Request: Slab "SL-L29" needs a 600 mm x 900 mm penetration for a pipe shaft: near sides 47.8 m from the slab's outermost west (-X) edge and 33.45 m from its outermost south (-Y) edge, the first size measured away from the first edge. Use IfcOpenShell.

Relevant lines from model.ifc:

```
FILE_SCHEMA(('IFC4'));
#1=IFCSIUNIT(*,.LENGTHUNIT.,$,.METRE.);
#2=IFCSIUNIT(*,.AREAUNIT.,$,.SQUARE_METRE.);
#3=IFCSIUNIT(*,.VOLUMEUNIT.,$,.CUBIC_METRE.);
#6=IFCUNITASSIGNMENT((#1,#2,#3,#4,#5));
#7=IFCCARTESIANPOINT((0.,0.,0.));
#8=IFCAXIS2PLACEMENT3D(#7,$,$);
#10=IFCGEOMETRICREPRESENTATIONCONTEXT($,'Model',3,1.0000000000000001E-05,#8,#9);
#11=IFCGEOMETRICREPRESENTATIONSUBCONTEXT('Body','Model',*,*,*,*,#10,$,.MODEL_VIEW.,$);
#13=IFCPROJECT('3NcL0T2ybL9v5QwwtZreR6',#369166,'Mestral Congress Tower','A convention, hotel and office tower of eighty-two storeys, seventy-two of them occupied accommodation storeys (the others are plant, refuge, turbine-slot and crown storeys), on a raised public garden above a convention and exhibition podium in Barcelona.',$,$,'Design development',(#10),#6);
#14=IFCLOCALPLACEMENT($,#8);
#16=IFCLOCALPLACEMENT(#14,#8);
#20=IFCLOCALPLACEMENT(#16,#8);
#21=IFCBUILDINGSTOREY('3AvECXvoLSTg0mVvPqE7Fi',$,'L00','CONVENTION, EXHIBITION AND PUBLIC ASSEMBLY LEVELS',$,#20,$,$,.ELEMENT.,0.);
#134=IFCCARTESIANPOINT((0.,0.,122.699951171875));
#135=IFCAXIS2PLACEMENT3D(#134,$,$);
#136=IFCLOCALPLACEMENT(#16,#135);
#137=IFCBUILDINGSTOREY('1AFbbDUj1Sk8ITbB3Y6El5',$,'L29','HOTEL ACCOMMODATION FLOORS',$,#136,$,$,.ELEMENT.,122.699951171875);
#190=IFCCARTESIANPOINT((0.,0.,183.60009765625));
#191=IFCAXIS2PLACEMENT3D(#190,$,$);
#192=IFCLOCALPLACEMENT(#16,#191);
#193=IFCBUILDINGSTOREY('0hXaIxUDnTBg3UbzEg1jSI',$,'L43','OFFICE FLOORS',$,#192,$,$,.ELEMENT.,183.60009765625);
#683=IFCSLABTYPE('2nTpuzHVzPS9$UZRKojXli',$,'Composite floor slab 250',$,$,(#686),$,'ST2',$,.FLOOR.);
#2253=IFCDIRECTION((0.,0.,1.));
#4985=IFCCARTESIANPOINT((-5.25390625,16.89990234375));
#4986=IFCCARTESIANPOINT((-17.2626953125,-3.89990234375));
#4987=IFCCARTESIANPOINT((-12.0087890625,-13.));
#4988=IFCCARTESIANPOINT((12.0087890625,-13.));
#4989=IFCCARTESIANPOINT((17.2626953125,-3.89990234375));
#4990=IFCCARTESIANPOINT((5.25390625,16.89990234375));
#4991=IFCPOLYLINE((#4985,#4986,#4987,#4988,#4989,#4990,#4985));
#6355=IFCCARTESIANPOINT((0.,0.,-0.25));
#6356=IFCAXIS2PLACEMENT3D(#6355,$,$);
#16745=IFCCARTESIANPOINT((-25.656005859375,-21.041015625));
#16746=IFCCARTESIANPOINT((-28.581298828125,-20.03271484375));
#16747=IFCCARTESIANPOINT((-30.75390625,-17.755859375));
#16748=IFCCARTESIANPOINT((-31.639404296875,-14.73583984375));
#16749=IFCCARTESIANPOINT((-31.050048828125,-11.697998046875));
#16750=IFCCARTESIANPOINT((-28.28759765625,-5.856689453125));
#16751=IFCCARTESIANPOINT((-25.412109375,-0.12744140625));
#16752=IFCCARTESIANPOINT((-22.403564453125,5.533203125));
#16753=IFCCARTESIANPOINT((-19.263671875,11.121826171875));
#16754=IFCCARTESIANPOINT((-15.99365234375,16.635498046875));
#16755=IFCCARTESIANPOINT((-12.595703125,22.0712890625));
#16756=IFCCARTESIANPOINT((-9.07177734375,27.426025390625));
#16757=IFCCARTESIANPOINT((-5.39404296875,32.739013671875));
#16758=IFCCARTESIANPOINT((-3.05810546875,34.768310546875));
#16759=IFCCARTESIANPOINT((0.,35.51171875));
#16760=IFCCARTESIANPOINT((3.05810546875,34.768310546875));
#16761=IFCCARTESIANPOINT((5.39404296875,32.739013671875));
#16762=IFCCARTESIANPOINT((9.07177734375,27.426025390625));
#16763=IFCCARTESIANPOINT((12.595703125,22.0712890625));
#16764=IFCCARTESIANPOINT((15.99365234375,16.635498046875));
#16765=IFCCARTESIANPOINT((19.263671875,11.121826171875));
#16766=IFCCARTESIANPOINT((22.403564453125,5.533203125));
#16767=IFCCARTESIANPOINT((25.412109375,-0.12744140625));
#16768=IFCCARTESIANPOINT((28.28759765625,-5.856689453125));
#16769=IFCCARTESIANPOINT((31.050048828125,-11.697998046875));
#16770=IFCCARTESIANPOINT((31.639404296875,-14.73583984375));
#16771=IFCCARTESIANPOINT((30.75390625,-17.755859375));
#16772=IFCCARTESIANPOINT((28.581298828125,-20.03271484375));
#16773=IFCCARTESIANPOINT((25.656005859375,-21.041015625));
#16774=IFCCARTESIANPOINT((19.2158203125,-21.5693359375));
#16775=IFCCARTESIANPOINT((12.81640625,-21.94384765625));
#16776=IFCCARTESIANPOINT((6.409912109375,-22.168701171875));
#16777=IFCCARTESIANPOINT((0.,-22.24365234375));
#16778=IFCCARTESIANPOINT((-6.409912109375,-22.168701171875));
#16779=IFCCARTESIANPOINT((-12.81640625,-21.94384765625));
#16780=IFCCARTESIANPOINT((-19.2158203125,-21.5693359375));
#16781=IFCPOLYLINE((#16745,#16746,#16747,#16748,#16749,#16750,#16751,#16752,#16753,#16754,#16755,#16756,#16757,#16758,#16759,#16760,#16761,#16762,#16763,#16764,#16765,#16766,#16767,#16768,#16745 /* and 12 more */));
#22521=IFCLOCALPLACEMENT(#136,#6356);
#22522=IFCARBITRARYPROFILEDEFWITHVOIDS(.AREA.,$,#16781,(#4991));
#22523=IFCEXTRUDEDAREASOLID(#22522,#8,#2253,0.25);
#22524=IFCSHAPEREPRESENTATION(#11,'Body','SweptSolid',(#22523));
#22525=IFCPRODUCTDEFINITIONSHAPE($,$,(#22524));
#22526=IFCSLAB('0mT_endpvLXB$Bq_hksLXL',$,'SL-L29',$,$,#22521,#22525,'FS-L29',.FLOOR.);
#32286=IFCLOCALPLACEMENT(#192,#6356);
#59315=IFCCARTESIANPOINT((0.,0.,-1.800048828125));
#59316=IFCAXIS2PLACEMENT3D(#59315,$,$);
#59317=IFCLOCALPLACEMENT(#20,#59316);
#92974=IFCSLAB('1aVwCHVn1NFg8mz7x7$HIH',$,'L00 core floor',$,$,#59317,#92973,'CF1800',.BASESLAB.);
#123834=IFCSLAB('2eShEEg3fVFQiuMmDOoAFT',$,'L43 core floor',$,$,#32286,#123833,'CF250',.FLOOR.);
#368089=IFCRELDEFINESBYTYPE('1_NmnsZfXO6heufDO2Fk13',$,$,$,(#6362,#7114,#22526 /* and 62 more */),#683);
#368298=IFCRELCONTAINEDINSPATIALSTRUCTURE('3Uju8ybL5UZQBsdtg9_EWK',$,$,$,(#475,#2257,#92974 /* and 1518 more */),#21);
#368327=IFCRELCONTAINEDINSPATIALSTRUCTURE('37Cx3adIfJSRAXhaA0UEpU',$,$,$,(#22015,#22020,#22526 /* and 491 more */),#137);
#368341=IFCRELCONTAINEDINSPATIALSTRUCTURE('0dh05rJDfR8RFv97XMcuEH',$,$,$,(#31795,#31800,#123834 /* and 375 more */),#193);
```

```python
import numpy as np
import ifcopenshell
import ifcopenshell.api.feature
import ifcopenshell.api.geometry
import ifcopenshell.api.root
import ifcopenshell.geom
import ifcopenshell.util.placement
import ifcopenshell.util.representation
import ifcopenshell.util.shape
import ifcopenshell.util.unit

model = ifcopenshell.open("model.ifc")
unit_scale = ifcopenshell.util.unit.calculate_unit_scale(model)
settings = ifcopenshell.geom.settings()


def volume(element):
    """Net volume in cubic metres, openings subtracted."""
    shape = ifcopenshell.geom.create_shape(settings, element)
    return ifcopenshell.util.shape.get_volume(shape.geometry)


slab = model.by_guid("0mT_endpvLXB$Bq_hksLXL")
before = volume(slab)

# Extent in the slab's own axes, in metres. The edges named are its -X and -Y sides.
slab_shape = ifcopenshell.geom.create_shape(settings, slab)
vertices = ifcopenshell.util.shape.get_vertices(slab_shape.geometry)
x_min, y_min, bottom = vertices.min(axis=0)
top = vertices[:, 2].max()

opening = ifcopenshell.api.root.create_entity(model, ifc_class="IfcOpeningElement", name="Pipe shaft opening", predefined_type="OPENING")
context = ifcopenshell.util.representation.get_context(model, "Model", "Body", "MODEL_VIEW")
width, depth = 0.6, 0.9
outline = [(0.0, 0.0), (width, 0.0), (width, depth), (0.0, depth), (0.0, 0.0)]
# Overshoot both faces by 50 mm so the cut is clean.
shape = ifcopenshell.api.geometry.add_slab_representation(
    model, context=context, depth=top - bottom + 0.1, polyline=outline
)
ifcopenshell.api.geometry.assign_representation(model, product=opening, representation=shape)

matrix = ifcopenshell.util.placement.get_local_placement(slab.ObjectPlacement)
matrix[:, 3] = matrix @ np.append(np.array([x_min + 47.8, y_min + 33.45, bottom - 0.05]) / unit_scale, 1.0)
ifcopenshell.api.geometry.edit_object_placement(model, product=opening, matrix=matrix, is_si=False)
ifcopenshell.api.feature.add_feature(model, feature=opening, element=slab)

after = volume(slab)

print(f"slab volume {before:.3f} -> {after:.3f} m3")

model.write("model-out.ifc")
```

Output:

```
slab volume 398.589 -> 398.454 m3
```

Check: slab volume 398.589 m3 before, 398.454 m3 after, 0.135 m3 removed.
